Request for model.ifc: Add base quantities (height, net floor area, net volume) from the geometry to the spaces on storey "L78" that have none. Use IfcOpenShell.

First a look at what the model holds.

```python
import ifcopenshell
import ifcopenshell.util.element
import ifcopenshell.util.unit

model = ifcopenshell.open("model.ifc")
print(model.schema)
for unit_type in ("LENGTHUNIT", "AREAUNIT", "VOLUMEUNIT"):
    print(unit_type, ifcopenshell.util.unit.calculate_unit_scale(model, unit_type))
storey = next(s for s in model.by_type("IfcBuildingStorey") if s.Name == "L78")
spaces = [e for e in ifcopenshell.util.element.get_decomposition(storey) if e.is_a("IfcSpace")]
for e in sorted(spaces, key=lambda e: e.id()):
    print(e.id(), e.is_a(), e.Name, list(ifcopenshell.util.element.get_psets(e, qtos_only=True)), sep=" | ")
```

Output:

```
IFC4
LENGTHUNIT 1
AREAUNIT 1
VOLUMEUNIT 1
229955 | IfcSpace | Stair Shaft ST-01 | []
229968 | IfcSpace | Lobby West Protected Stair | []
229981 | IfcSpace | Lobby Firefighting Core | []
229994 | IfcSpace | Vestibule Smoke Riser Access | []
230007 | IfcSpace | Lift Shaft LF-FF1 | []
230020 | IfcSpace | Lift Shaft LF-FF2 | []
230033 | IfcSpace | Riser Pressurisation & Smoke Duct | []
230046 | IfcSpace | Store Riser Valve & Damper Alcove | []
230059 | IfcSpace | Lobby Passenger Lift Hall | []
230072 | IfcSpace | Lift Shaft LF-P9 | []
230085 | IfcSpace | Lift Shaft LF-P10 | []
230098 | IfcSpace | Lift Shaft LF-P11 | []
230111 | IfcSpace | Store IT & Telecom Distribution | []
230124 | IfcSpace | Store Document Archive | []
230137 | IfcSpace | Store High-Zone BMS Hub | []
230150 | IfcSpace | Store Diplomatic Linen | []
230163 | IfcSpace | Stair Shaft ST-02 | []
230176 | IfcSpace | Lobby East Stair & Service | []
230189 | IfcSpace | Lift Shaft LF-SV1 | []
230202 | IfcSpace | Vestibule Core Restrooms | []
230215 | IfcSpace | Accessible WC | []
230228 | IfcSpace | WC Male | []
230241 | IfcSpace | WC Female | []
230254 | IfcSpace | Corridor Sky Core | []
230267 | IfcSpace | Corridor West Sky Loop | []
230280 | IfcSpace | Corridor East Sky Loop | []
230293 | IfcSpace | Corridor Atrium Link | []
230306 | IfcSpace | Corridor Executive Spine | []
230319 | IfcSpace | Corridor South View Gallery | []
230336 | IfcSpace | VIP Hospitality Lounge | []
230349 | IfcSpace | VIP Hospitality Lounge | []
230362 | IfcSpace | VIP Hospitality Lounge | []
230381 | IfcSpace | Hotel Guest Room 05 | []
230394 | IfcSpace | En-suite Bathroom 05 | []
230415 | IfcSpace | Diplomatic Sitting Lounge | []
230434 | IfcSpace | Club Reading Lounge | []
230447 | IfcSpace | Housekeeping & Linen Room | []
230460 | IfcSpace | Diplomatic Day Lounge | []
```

```python
import ifcopenshell
import ifcopenshell.api.pset
import ifcopenshell.geom
import ifcopenshell.util.element
import ifcopenshell.util.shape
import ifcopenshell.util.unit

model = ifcopenshell.open("model.ifc")
unit_scale = ifcopenshell.util.unit.calculate_unit_scale(model)
area_scale = ifcopenshell.util.unit.calculate_unit_scale(model, "AREAUNIT")
volume_scale = ifcopenshell.util.unit.calculate_unit_scale(model, "VOLUMEUNIT")
settings = ifcopenshell.geom.settings()

storey = next(s for s in model.by_type("IfcBuildingStorey") if s.Name == "L78")
spaces = [e for e in ifcopenshell.util.element.get_decomposition(storey) if e.is_a("IfcSpace")]

for e in sorted(spaces, key=lambda e: e.id()):
    if ifcopenshell.util.element.get_psets(e, qtos_only=True, should_inherit=False):
        continue
    # Geometry comes back in metres, in the element's own axes.
    shape = ifcopenshell.geom.create_shape(settings, e)
    values = {
        "Height": ifcopenshell.util.shape.get_z(shape.geometry) / unit_scale,
        "NetFloorArea": ifcopenshell.util.shape.get_footprint_area(shape.geometry) / area_scale,
        "NetVolume": ifcopenshell.util.shape.get_volume(shape.geometry) / volume_scale,
    }
    qto = ifcopenshell.api.pset.add_qto(model, product=e, name="Qto_SpaceBaseQuantities")
    ifcopenshell.api.pset.edit_qto(model, qto=qto, properties=values)
    print(e.id(), {k: round(v, 3) for k, v in values.items()})

model.write("model_updated.ifc")
```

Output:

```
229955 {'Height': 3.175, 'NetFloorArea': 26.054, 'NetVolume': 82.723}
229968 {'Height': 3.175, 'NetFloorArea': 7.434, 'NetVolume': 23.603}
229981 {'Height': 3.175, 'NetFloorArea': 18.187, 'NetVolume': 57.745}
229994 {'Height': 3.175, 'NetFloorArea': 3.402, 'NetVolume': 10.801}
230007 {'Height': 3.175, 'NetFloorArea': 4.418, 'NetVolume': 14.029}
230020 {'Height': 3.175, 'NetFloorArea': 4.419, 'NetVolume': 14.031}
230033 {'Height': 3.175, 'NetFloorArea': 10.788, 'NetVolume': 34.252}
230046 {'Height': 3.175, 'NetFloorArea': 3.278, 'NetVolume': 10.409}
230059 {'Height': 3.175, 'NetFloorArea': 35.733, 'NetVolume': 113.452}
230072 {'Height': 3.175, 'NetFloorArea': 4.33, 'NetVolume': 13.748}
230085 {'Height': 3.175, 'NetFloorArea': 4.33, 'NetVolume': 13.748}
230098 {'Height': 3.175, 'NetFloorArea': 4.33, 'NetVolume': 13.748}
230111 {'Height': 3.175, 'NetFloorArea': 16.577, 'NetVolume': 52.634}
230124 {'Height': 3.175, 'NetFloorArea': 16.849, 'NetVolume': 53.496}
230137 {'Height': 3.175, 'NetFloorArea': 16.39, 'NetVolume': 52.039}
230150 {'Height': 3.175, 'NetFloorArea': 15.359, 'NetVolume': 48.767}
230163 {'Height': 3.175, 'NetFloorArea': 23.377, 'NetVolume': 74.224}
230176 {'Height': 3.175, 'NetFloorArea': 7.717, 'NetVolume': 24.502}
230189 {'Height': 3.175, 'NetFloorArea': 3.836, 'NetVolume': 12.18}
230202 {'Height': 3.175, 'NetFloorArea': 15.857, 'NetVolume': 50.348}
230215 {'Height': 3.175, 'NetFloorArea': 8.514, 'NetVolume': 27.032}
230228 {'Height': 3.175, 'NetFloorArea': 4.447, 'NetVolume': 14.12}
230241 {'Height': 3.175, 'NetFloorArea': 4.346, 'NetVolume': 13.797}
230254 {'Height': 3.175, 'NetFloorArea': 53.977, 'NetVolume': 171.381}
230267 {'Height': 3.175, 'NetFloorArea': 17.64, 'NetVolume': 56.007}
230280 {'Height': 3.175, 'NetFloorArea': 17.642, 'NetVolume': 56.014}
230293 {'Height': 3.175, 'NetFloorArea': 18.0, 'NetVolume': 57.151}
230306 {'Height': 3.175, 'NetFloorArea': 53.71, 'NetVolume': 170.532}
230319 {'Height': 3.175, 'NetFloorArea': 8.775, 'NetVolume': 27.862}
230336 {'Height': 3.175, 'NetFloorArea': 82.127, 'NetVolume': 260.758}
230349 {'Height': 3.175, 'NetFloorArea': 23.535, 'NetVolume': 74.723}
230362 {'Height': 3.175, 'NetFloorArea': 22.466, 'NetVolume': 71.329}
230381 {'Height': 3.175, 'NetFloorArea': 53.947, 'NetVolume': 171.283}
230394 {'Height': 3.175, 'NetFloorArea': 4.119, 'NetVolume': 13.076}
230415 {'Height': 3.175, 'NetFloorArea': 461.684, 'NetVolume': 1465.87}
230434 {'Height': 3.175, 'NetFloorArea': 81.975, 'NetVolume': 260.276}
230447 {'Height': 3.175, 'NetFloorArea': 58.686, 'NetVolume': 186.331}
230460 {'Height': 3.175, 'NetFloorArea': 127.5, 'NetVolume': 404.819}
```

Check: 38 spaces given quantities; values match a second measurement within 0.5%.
